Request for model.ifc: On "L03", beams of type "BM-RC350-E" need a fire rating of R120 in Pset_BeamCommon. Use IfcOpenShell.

First a look at what the model holds.

```python
import ifcopenshell
import ifcopenshell.util.element

model = ifcopenshell.open("model.ifc")
print(model.schema)
storey = next(s for s in model.by_type("IfcBuildingStorey") if s.Name == "L03")
beams = [e for e in ifcopenshell.util.element.get_decomposition(storey) if e.is_a("IfcBeam")]
seen = {}
for e in beams:
    element_type = ifcopenshell.util.element.get_type(e)
    key = (element_type.Name if element_type != e and element_type else None, ifcopenshell.util.element.get_pset(e, "Pset_BeamCommon", "FireRating"))
    seen[key] = seen.get(key, 0) + 1
for (name, value), count in sorted(seen.items(), key=str):
    print(count, "x", name, "|", value)
```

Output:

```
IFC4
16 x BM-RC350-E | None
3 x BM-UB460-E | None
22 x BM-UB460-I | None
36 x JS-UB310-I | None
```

```python
import ifcopenshell
import ifcopenshell.api.pset
import ifcopenshell.util.element

model = ifcopenshell.open("model.ifc")

storey = next(s for s in model.by_type("IfcBuildingStorey") if s.Name == "L03")
beams = [e for e in ifcopenshell.util.element.get_decomposition(storey) if e.is_a("IfcBeam")]

count = 0
for e in beams:
    element_type = ifcopenshell.util.element.get_type(e)
    if element_type in (None, e) or element_type.Name != "BM-RC350-E":
        continue
    # add_pset returns the element's existing set when there is one.
    pset = ifcopenshell.api.pset.add_pset(model, product=e, name="Pset_BeamCommon")
    ifcopenshell.api.pset.edit_pset(model, pset=pset, properties={"FireRating": "R120"})
    count += 1

print(count, "beams updated")

model.write("model-out.ifc")
```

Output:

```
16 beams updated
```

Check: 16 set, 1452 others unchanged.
